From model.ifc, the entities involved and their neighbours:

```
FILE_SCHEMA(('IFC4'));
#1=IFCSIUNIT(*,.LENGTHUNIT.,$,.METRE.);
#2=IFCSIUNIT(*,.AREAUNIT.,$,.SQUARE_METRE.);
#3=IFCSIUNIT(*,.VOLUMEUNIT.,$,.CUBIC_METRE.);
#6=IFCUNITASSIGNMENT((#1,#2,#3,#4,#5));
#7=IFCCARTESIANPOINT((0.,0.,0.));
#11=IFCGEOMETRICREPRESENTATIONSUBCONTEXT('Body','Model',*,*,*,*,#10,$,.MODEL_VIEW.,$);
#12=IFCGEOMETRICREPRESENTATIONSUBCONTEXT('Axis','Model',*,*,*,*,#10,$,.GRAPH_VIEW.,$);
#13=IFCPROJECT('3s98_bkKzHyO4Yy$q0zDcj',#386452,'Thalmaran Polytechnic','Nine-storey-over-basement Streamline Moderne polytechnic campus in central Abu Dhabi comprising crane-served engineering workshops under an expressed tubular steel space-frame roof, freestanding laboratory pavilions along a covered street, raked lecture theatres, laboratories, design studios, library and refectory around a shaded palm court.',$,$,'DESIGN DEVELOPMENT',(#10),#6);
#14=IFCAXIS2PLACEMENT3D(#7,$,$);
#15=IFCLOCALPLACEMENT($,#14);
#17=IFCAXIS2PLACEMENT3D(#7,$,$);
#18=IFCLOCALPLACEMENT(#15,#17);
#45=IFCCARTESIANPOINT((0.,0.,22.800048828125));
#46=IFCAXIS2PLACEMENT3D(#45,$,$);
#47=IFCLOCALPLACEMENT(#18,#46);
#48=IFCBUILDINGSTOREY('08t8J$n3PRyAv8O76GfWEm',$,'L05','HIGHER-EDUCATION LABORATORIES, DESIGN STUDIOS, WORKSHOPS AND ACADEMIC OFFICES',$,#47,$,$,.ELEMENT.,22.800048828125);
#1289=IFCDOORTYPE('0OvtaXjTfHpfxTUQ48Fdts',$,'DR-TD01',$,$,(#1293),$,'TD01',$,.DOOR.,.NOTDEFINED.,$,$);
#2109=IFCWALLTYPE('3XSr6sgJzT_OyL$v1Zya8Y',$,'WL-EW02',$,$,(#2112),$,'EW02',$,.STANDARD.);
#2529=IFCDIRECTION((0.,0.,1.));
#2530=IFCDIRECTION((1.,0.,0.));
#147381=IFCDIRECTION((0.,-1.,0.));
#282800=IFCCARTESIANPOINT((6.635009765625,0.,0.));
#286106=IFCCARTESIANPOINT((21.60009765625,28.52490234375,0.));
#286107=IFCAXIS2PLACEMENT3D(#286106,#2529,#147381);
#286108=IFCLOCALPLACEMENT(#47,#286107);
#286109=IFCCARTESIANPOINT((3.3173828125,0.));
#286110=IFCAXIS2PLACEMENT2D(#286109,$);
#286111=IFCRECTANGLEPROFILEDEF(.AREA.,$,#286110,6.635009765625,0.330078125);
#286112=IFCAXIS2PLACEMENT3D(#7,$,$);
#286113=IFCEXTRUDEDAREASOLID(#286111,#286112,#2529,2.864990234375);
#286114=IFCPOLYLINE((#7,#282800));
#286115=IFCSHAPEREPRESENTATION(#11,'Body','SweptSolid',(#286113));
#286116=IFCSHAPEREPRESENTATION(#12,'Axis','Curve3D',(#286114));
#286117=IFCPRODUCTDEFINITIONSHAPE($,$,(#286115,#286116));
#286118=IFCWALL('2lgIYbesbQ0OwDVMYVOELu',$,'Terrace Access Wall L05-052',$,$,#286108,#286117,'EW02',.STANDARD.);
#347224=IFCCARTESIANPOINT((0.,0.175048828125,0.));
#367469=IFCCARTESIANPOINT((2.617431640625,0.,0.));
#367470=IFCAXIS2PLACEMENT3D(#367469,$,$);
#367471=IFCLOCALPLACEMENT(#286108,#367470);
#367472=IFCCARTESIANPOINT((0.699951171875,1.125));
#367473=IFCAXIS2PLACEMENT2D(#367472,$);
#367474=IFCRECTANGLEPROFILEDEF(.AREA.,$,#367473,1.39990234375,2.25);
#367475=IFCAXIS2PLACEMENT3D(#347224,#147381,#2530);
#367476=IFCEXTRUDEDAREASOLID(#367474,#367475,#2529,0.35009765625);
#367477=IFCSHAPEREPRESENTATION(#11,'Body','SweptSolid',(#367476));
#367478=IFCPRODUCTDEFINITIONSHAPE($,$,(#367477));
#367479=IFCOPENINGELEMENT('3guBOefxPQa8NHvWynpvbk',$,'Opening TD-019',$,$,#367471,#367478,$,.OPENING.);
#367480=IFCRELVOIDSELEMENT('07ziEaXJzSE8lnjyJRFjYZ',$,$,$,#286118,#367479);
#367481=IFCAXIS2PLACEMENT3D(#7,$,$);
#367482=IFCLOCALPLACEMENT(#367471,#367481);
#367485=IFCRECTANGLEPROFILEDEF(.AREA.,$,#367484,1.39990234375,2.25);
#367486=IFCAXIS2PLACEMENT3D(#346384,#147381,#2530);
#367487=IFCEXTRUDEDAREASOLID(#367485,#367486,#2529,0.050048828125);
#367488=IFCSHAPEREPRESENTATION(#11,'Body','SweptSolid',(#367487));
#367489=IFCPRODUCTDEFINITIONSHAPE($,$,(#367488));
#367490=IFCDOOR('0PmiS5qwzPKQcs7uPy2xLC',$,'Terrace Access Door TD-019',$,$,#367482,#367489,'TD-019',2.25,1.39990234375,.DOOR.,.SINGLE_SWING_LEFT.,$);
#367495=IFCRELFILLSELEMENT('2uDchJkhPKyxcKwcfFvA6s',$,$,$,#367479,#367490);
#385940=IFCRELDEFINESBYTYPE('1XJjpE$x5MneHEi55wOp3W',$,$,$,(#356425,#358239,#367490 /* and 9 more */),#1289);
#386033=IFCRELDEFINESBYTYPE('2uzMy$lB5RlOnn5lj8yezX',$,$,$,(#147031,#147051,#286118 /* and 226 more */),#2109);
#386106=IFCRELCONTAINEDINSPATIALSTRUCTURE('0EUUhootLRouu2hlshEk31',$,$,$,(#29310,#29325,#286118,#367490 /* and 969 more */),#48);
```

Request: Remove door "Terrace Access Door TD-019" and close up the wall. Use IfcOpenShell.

```python
import ifcopenshell
import ifcopenshell.api.feature
import ifcopenshell.api.root
import ifcopenshell.geom
import ifcopenshell.util.shape

model = ifcopenshell.open("model.ifc")
settings = ifcopenshell.geom.settings()


def volume(element):
    """Net volume in cubic metres, openings subtracted."""
    shape = ifcopenshell.geom.create_shape(settings, element)
    return ifcopenshell.util.shape.get_volume(shape.geometry)


door = model.by_guid("0PmiS5qwzPKQcs7uPy2xLC")
opening = door.FillsVoids[0].RelatingOpeningElement
wall = opening.VoidsElements[0].RelatingBuildingElement
before = volume(wall)

ifcopenshell.api.root.remove_product(model, product=door)
ifcopenshell.api.feature.remove_feature(model, feature=opening)

after = volume(wall)

print(f"wall volume {before:.3f} -> {after:.3f} m3")

model.write("model_rev.ifc")
```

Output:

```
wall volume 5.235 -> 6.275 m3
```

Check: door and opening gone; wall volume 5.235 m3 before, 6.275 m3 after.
